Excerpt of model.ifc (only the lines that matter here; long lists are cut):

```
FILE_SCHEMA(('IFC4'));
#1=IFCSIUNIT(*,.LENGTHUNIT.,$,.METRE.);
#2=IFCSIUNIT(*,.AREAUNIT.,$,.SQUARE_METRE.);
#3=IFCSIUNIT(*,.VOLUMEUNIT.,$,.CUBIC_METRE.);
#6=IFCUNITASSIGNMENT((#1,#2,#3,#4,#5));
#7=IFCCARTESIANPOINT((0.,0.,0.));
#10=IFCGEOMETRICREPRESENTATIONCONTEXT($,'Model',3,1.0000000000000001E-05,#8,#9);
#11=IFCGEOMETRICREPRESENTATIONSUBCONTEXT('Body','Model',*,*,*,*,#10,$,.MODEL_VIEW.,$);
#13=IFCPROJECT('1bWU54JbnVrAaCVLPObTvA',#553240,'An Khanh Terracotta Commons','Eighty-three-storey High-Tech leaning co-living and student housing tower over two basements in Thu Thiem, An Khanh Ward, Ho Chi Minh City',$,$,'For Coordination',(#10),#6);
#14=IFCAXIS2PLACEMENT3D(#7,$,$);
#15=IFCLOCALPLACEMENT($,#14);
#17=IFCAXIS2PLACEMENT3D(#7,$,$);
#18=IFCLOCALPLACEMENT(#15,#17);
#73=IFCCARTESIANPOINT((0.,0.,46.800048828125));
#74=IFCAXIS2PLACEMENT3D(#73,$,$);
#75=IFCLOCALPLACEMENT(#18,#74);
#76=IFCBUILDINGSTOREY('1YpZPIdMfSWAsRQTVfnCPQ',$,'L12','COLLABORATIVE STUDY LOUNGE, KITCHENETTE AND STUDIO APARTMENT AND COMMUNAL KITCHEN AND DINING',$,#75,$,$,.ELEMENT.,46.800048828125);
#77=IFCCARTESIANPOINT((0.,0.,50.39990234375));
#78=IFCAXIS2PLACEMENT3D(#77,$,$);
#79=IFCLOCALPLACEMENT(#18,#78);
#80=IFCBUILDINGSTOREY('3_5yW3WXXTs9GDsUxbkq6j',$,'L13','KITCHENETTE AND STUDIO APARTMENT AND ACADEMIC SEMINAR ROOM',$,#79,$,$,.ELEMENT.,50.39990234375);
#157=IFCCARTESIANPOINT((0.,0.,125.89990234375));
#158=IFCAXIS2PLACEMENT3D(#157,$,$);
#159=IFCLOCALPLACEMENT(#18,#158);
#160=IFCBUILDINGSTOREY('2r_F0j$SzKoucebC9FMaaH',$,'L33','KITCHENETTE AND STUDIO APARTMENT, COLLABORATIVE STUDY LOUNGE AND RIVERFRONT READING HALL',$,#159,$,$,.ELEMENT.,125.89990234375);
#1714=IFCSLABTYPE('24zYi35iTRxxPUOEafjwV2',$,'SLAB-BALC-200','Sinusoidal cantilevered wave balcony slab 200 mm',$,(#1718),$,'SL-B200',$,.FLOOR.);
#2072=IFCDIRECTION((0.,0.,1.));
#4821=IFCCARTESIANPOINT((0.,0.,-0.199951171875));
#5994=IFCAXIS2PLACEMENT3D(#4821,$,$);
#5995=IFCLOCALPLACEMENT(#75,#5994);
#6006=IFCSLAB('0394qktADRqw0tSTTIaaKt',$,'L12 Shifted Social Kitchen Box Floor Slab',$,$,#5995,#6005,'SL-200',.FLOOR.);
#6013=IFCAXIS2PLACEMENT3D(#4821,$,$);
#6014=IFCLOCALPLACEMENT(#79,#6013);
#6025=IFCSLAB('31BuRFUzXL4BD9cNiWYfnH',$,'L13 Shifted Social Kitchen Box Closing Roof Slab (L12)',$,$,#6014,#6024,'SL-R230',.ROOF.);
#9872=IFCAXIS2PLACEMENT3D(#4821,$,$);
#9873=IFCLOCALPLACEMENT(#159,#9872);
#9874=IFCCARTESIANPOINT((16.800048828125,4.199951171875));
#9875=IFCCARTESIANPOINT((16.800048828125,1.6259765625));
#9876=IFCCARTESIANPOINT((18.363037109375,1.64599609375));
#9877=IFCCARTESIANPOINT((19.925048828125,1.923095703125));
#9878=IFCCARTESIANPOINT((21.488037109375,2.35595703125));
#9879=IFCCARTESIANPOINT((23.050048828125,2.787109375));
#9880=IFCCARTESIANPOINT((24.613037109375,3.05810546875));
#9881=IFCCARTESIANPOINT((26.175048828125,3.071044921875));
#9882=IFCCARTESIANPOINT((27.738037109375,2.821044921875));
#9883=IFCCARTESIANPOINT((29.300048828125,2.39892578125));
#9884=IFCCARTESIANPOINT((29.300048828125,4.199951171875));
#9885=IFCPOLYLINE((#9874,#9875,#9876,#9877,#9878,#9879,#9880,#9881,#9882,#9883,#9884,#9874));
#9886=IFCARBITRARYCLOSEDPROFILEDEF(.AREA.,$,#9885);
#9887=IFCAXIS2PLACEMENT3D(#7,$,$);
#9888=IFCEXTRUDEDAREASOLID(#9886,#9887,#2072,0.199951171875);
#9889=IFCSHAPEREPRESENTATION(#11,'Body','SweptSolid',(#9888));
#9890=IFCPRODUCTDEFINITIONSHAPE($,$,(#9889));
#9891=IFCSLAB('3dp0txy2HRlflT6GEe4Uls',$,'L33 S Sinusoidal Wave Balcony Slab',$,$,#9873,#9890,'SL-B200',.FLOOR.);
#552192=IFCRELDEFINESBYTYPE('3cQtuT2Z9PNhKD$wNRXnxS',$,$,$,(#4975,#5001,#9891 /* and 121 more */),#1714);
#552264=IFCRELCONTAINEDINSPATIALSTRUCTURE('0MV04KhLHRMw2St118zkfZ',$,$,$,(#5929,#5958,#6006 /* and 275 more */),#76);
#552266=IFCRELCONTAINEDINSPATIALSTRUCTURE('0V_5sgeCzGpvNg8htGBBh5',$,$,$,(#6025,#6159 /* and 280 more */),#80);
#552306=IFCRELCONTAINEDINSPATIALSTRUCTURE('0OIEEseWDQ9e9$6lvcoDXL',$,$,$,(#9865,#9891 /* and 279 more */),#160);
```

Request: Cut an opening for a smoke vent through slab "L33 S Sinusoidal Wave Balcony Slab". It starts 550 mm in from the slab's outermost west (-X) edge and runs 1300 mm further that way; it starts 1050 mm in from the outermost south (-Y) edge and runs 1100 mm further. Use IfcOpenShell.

```python
import numpy as np
import ifcopenshell
import ifcopenshell.api.feature
import ifcopenshell.api.geometry
import ifcopenshell.api.root
import ifcopenshell.geom
import ifcopenshell.util.placement
import ifcopenshell.util.representation
import ifcopenshell.util.shape
import ifcopenshell.util.unit

model = ifcopenshell.open("model.ifc")
unit_scale = ifcopenshell.util.unit.calculate_unit_scale(model)
settings = ifcopenshell.geom.settings()


def volume(element):
    """Net volume in cubic metres, openings subtracted."""
    shape = ifcopenshell.geom.create_shape(settings, element)
    return ifcopenshell.util.shape.get_volume(shape.geometry)


slab = model.by_guid("3dp0txy2HRlflT6GEe4Uls")
before = volume(slab)

# Extent in the slab's own axes, in metres. The edges named are its -X and -Y sides.
slab_shape = ifcopenshell.geom.create_shape(settings, slab)
vertices = ifcopenshell.util.shape.get_vertices(slab_shape.geometry)
x_min, y_min, bottom = vertices.min(axis=0)
top = vertices[:, 2].max()

opening = ifcopenshell.api.root.create_entity(model, ifc_class="IfcOpeningElement", name="Smoke vent opening", predefined_type="OPENING")
context = ifcopenshell.util.representation.get_context(model, "Model", "Body", "MODEL_VIEW")
width, depth = 1.3, 1.1
outline = [(0.0, 0.0), (width, 0.0), (width, depth), (0.0, depth), (0.0, 0.0)]
# Overshoot both faces by 50 mm so the cut is clean.
shape = ifcopenshell.api.geometry.add_slab_representation(
    model, context=context, depth=top - bottom + 0.1, polyline=outline
)
ifcopenshell.api.geometry.assign_representation(model, product=opening, representation=shape)

matrix = ifcopenshell.util.placement.get_local_placement(slab.ObjectPlacement)
matrix[:, 3] = matrix @ np.append(np.array([x_min + 0.55, y_min + 1.05, bottom - 0.05]) / unit_scale, 1.0)
ifcopenshell.api.geometry.edit_object_placement(model, product=opening, matrix=matrix, is_si=False)
ifcopenshell.api.feature.add_feature(model, feature=opening, element=slab)

after = volume(slab)

print(f"slab volume {before:.3f} -> {after:.3f} m3")

model.write("model_rev.ifc")
```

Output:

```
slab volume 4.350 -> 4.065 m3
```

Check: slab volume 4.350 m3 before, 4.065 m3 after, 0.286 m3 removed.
